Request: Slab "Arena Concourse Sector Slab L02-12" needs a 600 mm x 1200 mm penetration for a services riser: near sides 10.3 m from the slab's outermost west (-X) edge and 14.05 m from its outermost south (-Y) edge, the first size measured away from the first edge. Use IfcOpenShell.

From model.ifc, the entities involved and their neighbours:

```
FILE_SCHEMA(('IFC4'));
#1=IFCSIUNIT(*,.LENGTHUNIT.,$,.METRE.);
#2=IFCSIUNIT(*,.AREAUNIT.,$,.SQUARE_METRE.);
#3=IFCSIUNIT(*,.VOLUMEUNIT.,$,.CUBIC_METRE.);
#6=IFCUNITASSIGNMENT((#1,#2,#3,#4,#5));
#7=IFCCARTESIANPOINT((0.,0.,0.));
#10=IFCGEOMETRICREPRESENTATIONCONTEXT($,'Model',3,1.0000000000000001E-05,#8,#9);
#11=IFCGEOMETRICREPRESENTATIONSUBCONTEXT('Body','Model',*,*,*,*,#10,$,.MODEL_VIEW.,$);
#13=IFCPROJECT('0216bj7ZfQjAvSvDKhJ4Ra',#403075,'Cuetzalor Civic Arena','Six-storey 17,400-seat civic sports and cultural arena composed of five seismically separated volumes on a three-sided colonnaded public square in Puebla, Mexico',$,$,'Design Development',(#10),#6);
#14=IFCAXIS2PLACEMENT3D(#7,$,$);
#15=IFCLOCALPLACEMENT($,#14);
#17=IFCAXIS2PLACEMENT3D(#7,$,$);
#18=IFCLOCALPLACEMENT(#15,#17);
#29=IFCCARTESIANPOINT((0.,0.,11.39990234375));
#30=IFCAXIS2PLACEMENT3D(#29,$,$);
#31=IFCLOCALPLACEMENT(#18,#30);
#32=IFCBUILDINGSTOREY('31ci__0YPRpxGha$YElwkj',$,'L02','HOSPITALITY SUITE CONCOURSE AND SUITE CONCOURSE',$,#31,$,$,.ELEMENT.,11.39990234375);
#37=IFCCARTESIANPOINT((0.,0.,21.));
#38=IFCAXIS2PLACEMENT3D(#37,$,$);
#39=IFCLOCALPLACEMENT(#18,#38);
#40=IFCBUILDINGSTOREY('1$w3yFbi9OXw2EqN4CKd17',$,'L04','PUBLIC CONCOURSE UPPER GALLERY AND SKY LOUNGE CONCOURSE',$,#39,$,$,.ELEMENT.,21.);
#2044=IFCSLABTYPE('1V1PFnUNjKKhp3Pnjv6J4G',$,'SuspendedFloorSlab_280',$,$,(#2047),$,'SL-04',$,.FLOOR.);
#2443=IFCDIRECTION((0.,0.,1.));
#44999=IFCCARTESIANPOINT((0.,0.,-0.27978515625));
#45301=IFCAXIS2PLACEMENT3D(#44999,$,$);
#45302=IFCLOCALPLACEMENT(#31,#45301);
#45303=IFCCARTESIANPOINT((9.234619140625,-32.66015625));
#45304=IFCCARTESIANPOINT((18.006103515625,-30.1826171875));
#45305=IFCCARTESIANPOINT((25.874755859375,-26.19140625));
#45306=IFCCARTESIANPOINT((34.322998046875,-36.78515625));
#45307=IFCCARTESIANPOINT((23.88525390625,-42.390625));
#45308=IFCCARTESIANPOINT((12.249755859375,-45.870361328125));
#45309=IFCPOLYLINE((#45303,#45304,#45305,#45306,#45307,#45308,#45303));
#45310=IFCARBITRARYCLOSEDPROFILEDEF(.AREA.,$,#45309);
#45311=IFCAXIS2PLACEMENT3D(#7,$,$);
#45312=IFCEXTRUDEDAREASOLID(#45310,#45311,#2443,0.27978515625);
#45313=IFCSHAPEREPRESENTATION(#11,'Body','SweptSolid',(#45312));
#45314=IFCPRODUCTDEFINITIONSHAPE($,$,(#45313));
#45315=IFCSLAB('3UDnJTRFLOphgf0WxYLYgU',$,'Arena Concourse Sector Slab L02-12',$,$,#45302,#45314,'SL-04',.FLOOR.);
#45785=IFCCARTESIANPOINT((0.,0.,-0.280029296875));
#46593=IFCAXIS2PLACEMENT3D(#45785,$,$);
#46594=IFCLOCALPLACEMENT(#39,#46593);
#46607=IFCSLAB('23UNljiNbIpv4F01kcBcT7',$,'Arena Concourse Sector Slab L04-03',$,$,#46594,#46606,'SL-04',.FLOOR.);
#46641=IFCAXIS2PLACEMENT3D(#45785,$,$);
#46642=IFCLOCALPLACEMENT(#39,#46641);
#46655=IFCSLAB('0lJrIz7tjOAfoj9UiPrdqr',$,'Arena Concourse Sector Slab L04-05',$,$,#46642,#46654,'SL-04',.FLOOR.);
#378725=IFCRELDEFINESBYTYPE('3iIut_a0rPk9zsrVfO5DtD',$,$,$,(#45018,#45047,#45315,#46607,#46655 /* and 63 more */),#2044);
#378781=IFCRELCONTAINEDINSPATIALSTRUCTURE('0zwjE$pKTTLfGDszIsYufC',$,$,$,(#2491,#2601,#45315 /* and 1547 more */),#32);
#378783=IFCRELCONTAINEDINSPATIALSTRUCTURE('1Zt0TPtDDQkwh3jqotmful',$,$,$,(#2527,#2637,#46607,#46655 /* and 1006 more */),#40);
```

```python
import numpy as np
import ifcopenshell
import ifcopenshell.api.feature
import ifcopenshell.api.geometry
import ifcopenshell.api.root
import ifcopenshell.geom
import ifcopenshell.util.placement
import ifcopenshell.util.representation
import ifcopenshell.util.shape
import ifcopenshell.util.unit

model = ifcopenshell.open("model.ifc")
unit_scale = ifcopenshell.util.unit.calculate_unit_scale(model)
settings = ifcopenshell.geom.settings()


def volume(element):
    """Net volume in cubic metres, openings subtracted."""
    shape = ifcopenshell.geom.create_shape(settings, element)
    return ifcopenshell.util.shape.get_volume(shape.geometry)


slab = model.by_guid("3UDnJTRFLOphgf0WxYLYgU")
before = volume(slab)

# Extent in the slab's own axes, in metres. The edges named are its -X and -Y sides.
slab_shape = ifcopenshell.geom.create_shape(settings, slab)
vertices = ifcopenshell.util.shape.get_vertices(slab_shape.geometry)
x_min, y_min, bottom = vertices.min(axis=0)
top = vertices[:, 2].max()

opening = ifcopenshell.api.root.create_entity(model, ifc_class="IfcOpeningElement", name="Services riser opening", predefined_type="OPENING")
context = ifcopenshell.util.representation.get_context(model, "Model", "Body", "MODEL_VIEW")
width, depth = 0.6, 1.2
outline = [(0.0, 0.0), (width, 0.0), (width, depth), (0.0, depth), (0.0, 0.0)]
# Overshoot both faces by 50 mm so the cut is clean.
shape = ifcopenshell.api.geometry.add_slab_representation(
    model, context=context, depth=top - bottom + 0.1, polyline=outline
)
ifcopenshell.api.geometry.assign_representation(model, product=opening, representation=shape)

matrix = ifcopenshell.util.placement.get_local_placement(slab.ObjectPlacement)
matrix[:, 3] = matrix @ np.append(np.array([x_min + 10.3, y_min + 14.05, bottom - 0.05]) / unit_scale, 1.0)
ifcopenshell.api.geometry.edit_object_placement(model, product=opening, matrix=matrix, is_si=False)
ifcopenshell.api.feature.add_feature(model, feature=opening, element=slab)

after = volume(slab)

print(f"slab volume {before:.3f} -> {after:.3f} m3")

model.write("model-out.ifc")
```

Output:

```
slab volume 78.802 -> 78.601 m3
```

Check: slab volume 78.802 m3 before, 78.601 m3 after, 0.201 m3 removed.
